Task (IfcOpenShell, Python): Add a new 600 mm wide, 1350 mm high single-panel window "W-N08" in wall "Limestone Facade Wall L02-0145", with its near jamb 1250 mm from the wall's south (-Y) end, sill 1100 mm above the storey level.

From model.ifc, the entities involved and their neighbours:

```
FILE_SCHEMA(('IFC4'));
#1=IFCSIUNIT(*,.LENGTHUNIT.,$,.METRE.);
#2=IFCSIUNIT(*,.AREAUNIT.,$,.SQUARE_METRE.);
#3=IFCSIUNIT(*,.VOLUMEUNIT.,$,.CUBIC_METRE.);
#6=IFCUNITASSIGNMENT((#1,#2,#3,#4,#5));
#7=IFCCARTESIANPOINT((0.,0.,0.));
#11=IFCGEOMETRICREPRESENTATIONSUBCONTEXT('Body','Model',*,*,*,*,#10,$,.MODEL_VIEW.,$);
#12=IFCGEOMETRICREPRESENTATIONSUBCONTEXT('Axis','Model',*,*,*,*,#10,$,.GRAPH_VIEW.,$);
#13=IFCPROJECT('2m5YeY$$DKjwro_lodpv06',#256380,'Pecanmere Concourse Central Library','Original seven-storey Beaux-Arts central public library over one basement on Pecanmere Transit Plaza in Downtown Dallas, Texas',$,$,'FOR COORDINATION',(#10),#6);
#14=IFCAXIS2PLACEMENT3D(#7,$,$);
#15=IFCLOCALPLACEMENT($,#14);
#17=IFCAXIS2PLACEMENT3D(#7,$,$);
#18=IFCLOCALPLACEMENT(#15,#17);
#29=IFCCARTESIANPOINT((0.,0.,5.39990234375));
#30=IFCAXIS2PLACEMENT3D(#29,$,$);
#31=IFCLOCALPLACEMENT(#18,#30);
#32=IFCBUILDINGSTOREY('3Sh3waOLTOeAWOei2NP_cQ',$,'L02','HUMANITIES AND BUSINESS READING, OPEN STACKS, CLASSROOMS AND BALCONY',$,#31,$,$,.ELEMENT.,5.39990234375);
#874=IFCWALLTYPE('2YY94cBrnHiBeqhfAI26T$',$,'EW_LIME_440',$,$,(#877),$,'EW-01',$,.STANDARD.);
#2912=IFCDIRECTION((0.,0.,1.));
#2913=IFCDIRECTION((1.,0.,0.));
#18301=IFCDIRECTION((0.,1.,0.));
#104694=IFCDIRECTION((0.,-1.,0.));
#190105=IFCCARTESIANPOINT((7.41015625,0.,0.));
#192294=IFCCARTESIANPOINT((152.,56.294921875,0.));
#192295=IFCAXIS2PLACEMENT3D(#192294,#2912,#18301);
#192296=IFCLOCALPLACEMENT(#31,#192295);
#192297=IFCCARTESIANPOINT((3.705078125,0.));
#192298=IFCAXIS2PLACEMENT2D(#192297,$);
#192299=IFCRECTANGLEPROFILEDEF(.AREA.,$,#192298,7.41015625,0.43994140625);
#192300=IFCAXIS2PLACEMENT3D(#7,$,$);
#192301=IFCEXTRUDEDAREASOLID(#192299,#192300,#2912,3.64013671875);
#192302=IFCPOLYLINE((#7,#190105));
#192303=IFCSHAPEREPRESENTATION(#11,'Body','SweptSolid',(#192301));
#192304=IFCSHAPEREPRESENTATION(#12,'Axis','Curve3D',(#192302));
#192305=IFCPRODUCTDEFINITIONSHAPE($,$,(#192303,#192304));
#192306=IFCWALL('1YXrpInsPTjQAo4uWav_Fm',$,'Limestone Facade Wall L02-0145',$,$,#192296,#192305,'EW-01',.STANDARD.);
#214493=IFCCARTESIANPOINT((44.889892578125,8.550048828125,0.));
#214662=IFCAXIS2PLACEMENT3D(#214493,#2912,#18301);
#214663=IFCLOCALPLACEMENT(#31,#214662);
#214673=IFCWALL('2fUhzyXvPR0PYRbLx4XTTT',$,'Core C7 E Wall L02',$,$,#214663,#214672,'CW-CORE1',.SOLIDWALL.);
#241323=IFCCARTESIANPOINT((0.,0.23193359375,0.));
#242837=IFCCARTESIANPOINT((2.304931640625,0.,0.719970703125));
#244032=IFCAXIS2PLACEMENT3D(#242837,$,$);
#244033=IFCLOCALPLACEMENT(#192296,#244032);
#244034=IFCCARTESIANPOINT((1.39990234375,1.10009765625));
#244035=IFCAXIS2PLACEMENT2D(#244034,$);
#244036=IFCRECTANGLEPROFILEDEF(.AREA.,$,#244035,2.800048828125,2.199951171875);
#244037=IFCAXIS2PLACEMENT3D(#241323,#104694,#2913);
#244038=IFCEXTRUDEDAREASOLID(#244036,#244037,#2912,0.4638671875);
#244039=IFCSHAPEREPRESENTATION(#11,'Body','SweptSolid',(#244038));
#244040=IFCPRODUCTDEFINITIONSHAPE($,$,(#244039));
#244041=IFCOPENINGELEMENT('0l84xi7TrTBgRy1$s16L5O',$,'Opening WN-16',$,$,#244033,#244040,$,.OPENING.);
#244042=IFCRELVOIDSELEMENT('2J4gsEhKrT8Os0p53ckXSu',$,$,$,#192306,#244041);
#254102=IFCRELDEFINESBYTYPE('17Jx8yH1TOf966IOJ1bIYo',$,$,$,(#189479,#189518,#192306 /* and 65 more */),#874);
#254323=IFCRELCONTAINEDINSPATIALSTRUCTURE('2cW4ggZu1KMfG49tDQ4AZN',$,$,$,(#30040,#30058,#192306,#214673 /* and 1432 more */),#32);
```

```python
import numpy as np
import ifcopenshell
import ifcopenshell.api.feature
import ifcopenshell.api.geometry
import ifcopenshell.api.root
import ifcopenshell.api.spatial
import ifcopenshell.geom
import ifcopenshell.util.element
import ifcopenshell.util.placement
import ifcopenshell.util.representation
import ifcopenshell.util.shape
import ifcopenshell.util.unit

model = ifcopenshell.open("model.ifc")
unit_scale = ifcopenshell.util.unit.calculate_unit_scale(model)
settings = ifcopenshell.geom.settings()


def volume(element):
    """Net volume in cubic metres, openings subtracted."""
    shape = ifcopenshell.geom.create_shape(settings, element)
    return ifcopenshell.util.shape.get_volume(shape.geometry)


wall = model.by_guid("1YXrpInsPTjQAo4uWav_Fm")
storey = ifcopenshell.util.element.get_container(wall, ifc_class="IfcBuildingStorey")
context = ifcopenshell.util.representation.get_context(model, "Model", "Body", "MODEL_VIEW")
before = volume(wall)

width, height, from_end, sill = 0.6, 1.35, 1.25, 1.1  # metres

# The wall runs along its own X axis, and the end named is its -X end.
wall_shape = ifcopenshell.geom.create_shape(settings, wall)
x, y, z = ifcopenshell.util.shape.get_vertices(wall_shape.geometry).T
start = x.min() + from_end
face, thickness = float(y.min()), float(y.max() - y.min())
wall_matrix = ifcopenshell.util.placement.get_local_placement(wall.ObjectPlacement)
level = ifcopenshell.util.placement.get_local_placement(storey.ObjectPlacement)[2, 3]


def in_wall(x, y):
    """Placement at x, y metres in the wall's axes, at sill height."""
    matrix = wall_matrix.copy()
    matrix[:, 3] = wall_matrix @ np.array([x / unit_scale, y / unit_scale, 0.0, 1.0])
    matrix[2, 3] = level + sill / unit_scale
    return matrix


# Opening: a box that overshoots both wall faces by 50 mm.
opening = ifcopenshell.api.root.create_entity(model, ifc_class="IfcOpeningElement", predefined_type="OPENING")
box = ifcopenshell.api.geometry.add_wall_representation(
    model, context=context, length=width, height=height, thickness=thickness + 0.1
)
ifcopenshell.api.geometry.assign_representation(model, product=opening, representation=box)
ifcopenshell.api.geometry.edit_object_placement(model, product=opening, matrix=in_wall(start, face - 0.05), is_si=False)
ifcopenshell.api.feature.add_feature(model, feature=opening, element=wall)

window = ifcopenshell.api.root.create_entity(model, ifc_class="IfcWindow", name="W-N08", predefined_type="WINDOW")
window.OverallWidth, window.OverallHeight = width / unit_scale, height / unit_scale
window.PartitioningType = "SINGLE_PANEL"
body = ifcopenshell.api.geometry.add_window_representation(
    model,
    context=context,
    overall_width=window.OverallWidth,
    overall_height=window.OverallHeight,
    partition_type="SINGLE_PANEL",
)
ifcopenshell.api.geometry.assign_representation(model, product=window, representation=body)
ifcopenshell.api.spatial.assign_container(model, products=[window], relating_structure=storey)
ifcopenshell.api.feature.add_filling(model, opening=opening, element=window)

# Centre the window in the wall's thickness.
ifcopenshell.api.geometry.edit_object_placement(model, product=window, matrix=in_wall(start, face), is_si=False)
window_shape = ifcopenshell.geom.create_shape(settings, window)
depth = ifcopenshell.util.shape.get_vertices(window_shape.geometry)[:, 1]
offset = face + thickness / 2 - (depth.min() + depth.max()) / 2
ifcopenshell.api.geometry.edit_object_placement(model, product=window, matrix=in_wall(start, offset), is_si=False)

after = volume(wall)

print(f"wall volume {before:.3f} -> {after:.3f} m3")

model.write("model_rev.ifc")
```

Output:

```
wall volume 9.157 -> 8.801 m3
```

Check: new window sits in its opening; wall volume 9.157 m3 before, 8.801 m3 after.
